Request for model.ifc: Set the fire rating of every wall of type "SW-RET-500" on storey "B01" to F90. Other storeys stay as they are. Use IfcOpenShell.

First a look at what the model holds.

```python
import ifcopenshell
import ifcopenshell.util.element

model = ifcopenshell.open("model.ifc")
print(model.schema)
storey = next(s for s in model.by_type("IfcBuildingStorey") if s.Name == "B01")
walls = [e for e in ifcopenshell.util.element.get_decomposition(storey) if e.is_a("IfcWall")]
seen = {}
for e in walls:
    element_type = ifcopenshell.util.element.get_type(e)
    key = (element_type.Name if element_type != e and element_type else None, ifcopenshell.util.element.get_pset(e, "Pset_WallCommon", "FireRating"))
    seen[key] = seen.get(key, 0) + 1
for (name, value), count in sorted(seen.items(), key=str):
    print(count, "x", name, "|", value)
```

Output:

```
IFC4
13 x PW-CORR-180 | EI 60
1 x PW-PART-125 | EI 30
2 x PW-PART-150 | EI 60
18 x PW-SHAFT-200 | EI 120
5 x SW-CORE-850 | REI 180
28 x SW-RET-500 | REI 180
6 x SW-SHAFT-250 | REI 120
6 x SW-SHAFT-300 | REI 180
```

```python
import ifcopenshell
import ifcopenshell.api.pset
import ifcopenshell.util.element

model = ifcopenshell.open("model.ifc")

storey = next(s for s in model.by_type("IfcBuildingStorey") if s.Name == "B01")
walls = [e for e in ifcopenshell.util.element.get_decomposition(storey) if e.is_a("IfcWall")]

count = 0
for e in walls:
    element_type = ifcopenshell.util.element.get_type(e)
    if element_type in (None, e) or element_type.Name != "SW-RET-500":
        continue
    found = ifcopenshell.util.element.get_pset(e, "Pset_WallCommon", should_inherit=False)
    if found:
        pset = model.by_id(found["id"])
        if len(ifcopenshell.util.element.get_elements_by_pset(pset)) > 1:
            pset = ifcopenshell.api.pset.unshare_pset(model, products=[e], pset=pset)[0]
    else:
        pset = ifcopenshell.api.pset.add_pset(model, product=e, name="Pset_WallCommon")
    ifcopenshell.api.pset.edit_pset(model, pset=pset, properties={"FireRating": "F90"})
    count += 1

print(count, "walls updated")

model.write("model_updated.ifc")
```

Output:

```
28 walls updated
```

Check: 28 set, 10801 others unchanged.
